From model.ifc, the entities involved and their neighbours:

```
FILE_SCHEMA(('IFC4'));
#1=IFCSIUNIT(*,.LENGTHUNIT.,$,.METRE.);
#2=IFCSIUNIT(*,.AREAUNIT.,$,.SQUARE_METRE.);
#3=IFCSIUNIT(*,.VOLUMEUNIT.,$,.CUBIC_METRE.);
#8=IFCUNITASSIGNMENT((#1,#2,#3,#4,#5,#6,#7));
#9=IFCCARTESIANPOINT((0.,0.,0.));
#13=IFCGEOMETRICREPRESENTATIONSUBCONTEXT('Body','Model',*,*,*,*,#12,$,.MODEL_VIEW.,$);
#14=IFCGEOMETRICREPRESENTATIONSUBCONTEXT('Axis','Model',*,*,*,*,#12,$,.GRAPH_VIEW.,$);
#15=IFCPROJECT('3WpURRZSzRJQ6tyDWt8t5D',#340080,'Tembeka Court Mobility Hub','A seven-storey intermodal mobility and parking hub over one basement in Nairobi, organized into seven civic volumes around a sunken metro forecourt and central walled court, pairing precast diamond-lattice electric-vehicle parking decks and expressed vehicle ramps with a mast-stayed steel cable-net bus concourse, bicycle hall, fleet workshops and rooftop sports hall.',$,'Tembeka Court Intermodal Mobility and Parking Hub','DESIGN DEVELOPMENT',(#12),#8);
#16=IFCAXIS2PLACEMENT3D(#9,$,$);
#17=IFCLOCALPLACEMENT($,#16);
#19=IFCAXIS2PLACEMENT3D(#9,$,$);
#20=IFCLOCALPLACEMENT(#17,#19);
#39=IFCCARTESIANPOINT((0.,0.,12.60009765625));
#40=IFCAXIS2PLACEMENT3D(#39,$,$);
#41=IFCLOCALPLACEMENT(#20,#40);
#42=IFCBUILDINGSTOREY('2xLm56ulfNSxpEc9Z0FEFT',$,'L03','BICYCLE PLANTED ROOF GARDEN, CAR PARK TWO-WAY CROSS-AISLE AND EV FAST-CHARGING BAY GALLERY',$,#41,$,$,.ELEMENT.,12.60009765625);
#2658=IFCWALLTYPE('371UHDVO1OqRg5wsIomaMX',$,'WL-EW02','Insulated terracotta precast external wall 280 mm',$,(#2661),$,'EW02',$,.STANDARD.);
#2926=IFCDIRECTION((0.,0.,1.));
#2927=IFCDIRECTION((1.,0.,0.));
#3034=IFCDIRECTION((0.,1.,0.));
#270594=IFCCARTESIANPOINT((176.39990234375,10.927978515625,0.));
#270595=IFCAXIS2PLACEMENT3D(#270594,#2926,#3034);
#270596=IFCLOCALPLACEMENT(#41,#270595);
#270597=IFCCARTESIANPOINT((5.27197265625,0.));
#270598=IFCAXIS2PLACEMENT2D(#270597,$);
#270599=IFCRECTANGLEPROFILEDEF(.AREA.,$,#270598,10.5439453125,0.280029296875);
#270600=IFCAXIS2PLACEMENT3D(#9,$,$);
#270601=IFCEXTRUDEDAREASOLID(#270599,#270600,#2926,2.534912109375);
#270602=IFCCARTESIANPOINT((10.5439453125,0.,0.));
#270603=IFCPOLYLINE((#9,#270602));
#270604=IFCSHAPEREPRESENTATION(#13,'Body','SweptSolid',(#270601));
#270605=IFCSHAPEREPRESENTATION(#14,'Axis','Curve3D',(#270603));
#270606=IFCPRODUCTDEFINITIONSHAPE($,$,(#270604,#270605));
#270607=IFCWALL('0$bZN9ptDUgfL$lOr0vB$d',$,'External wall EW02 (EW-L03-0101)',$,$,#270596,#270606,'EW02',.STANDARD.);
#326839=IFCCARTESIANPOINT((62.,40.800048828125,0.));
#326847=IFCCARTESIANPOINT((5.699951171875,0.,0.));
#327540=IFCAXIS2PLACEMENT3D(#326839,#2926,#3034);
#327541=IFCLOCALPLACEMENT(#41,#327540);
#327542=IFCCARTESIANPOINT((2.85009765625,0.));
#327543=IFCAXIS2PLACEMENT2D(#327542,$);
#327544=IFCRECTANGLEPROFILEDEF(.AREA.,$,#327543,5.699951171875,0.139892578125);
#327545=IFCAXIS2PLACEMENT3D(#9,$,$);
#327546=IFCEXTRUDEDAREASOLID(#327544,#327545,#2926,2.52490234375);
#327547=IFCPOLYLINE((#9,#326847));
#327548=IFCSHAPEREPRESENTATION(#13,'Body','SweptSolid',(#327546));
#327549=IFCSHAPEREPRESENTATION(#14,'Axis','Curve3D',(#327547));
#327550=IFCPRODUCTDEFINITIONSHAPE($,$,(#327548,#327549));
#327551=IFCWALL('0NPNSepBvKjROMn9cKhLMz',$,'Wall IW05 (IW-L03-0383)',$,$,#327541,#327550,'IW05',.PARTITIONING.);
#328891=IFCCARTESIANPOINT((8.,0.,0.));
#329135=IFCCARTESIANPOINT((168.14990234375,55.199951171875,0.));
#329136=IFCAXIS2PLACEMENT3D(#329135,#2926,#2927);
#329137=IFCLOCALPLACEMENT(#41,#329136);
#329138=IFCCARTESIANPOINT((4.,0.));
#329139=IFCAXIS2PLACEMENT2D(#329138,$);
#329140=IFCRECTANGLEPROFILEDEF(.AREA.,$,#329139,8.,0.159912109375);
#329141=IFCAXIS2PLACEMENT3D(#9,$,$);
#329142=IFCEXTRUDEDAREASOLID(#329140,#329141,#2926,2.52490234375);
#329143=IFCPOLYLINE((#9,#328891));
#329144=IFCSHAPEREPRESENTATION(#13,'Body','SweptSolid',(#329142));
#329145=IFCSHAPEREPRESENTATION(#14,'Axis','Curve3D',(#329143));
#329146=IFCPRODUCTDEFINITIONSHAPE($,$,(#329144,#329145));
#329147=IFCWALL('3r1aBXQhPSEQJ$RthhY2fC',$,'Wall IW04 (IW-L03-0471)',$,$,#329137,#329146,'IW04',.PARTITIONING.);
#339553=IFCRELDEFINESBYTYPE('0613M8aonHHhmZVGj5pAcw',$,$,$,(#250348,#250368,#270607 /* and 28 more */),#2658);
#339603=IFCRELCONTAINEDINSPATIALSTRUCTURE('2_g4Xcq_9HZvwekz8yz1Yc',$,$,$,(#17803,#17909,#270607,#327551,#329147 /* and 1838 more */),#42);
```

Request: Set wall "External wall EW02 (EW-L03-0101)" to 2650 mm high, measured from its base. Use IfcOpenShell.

```python
import ifcopenshell
import ifcopenshell.geom
import ifcopenshell.util.representation
import ifcopenshell.util.shape
import ifcopenshell.util.unit

model = ifcopenshell.open("model.ifc")
unit_scale = ifcopenshell.util.unit.calculate_unit_scale(model)
settings = ifcopenshell.geom.settings()


def volume(element):
    """Net volume in cubic metres, openings subtracted."""
    shape = ifcopenshell.geom.create_shape(settings, element)
    return ifcopenshell.util.shape.get_volume(shape.geometry)


wall = model.by_id(270607)
before = volume(wall)

body = ifcopenshell.util.representation.get_representation(wall, "Model", "Body")
solid = body.Items[0]
old_height = solid.Depth
solid.Depth = 2.65 / unit_scale
after = volume(wall)

print(f"height {old_height:g} -> {solid.Depth:g}, volume {before:.3f} -> {after:.3f} m3")

model.write("model-out.ifc")
```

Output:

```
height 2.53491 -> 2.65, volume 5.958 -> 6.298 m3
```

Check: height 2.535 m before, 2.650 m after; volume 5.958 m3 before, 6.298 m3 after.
